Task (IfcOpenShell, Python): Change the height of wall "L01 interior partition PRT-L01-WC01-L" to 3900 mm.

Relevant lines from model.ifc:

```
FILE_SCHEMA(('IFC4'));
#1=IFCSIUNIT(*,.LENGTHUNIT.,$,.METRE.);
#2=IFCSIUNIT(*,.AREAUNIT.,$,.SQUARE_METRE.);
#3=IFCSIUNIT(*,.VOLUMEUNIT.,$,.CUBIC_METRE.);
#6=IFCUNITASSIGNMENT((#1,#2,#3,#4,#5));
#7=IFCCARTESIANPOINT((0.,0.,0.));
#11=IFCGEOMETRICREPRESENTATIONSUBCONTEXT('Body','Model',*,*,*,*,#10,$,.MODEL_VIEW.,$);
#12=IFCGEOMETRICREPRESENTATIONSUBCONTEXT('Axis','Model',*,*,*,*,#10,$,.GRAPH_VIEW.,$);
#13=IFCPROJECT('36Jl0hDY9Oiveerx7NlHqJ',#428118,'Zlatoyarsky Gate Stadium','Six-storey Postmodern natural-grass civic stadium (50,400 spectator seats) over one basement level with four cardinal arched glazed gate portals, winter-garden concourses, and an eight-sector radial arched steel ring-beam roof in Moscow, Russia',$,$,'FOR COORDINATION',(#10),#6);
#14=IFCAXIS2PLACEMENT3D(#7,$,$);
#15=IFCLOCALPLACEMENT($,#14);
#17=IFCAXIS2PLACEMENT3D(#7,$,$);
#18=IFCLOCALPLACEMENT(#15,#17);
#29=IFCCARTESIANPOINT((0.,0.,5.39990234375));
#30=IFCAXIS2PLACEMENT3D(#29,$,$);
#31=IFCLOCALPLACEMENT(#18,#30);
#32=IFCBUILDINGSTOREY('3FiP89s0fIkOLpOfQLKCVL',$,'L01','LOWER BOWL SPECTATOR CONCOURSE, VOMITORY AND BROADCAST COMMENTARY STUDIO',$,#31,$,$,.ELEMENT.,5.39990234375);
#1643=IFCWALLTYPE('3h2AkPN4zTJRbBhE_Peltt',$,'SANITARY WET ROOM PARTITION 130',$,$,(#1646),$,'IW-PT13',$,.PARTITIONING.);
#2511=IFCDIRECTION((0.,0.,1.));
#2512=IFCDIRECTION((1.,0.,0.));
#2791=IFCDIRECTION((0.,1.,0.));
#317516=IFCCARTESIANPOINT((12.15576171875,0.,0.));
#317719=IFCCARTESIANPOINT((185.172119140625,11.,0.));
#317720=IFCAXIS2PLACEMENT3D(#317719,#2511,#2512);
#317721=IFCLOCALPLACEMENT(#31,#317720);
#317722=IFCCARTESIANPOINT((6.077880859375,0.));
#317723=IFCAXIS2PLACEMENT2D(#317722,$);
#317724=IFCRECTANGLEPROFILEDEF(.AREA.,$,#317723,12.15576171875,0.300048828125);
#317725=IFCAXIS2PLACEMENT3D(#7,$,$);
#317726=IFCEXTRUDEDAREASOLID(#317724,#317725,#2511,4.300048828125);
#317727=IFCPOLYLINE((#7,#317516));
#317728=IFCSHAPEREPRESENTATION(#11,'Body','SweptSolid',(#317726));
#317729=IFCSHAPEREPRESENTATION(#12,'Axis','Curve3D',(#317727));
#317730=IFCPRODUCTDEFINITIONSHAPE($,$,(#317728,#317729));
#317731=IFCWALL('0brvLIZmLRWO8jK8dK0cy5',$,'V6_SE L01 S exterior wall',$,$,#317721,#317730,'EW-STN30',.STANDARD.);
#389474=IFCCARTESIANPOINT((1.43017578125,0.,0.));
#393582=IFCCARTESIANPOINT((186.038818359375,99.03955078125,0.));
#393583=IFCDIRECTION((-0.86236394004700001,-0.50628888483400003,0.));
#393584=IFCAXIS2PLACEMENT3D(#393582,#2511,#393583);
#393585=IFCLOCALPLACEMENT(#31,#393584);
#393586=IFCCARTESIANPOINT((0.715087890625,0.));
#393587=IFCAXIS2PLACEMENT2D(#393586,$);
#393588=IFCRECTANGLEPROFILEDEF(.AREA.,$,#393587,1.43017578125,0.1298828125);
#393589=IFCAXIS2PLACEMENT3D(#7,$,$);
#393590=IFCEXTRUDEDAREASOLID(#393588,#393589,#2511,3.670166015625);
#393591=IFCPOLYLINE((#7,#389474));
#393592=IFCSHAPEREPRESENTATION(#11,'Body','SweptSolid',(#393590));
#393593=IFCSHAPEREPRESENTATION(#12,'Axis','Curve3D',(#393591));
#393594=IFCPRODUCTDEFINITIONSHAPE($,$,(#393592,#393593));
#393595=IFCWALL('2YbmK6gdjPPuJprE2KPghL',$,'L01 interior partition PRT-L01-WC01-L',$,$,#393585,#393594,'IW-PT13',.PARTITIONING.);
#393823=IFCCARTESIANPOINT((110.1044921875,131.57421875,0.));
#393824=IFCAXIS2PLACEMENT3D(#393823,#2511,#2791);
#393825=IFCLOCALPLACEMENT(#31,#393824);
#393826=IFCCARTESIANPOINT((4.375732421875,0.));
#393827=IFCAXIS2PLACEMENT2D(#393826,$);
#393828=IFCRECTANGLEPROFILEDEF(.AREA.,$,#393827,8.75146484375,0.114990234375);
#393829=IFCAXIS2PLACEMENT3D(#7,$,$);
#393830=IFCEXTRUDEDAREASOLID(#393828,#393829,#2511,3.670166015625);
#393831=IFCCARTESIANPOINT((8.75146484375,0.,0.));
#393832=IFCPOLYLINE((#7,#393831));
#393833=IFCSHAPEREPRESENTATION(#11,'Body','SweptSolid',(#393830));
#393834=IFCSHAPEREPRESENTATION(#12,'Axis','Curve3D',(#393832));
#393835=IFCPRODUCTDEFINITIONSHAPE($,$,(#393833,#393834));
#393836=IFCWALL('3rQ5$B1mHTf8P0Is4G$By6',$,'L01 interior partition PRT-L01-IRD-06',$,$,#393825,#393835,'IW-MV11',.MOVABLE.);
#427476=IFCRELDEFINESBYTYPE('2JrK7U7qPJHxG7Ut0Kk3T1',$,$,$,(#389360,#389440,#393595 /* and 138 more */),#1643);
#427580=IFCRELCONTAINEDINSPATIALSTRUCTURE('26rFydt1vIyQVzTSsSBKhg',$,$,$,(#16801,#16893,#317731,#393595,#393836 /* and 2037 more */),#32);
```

```python
import ifcopenshell
import ifcopenshell.geom
import ifcopenshell.util.representation
import ifcopenshell.util.shape

model = ifcopenshell.open("model.ifc")
settings = ifcopenshell.geom.settings()


def volume(element):
    """Net volume in cubic metres, openings subtracted."""
    shape = ifcopenshell.geom.create_shape(settings, element)
    return ifcopenshell.util.shape.get_volume(shape.geometry)


wall = model.by_guid("2YbmK6gdjPPuJprE2KPghL")
before = volume(wall)

body = ifcopenshell.util.representation.get_representation(wall, "Model", "Body")
solid = body.Items[0]
old_height = solid.Depth
solid.Depth = 3.9
after = volume(wall)

print(f"height {old_height:g} -> {solid.Depth:g}, volume {before:.3f} -> {after:.3f} m3")

model.write("model_edited.ifc")
```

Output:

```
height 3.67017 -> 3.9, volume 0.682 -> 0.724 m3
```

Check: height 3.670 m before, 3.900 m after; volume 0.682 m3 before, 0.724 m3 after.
